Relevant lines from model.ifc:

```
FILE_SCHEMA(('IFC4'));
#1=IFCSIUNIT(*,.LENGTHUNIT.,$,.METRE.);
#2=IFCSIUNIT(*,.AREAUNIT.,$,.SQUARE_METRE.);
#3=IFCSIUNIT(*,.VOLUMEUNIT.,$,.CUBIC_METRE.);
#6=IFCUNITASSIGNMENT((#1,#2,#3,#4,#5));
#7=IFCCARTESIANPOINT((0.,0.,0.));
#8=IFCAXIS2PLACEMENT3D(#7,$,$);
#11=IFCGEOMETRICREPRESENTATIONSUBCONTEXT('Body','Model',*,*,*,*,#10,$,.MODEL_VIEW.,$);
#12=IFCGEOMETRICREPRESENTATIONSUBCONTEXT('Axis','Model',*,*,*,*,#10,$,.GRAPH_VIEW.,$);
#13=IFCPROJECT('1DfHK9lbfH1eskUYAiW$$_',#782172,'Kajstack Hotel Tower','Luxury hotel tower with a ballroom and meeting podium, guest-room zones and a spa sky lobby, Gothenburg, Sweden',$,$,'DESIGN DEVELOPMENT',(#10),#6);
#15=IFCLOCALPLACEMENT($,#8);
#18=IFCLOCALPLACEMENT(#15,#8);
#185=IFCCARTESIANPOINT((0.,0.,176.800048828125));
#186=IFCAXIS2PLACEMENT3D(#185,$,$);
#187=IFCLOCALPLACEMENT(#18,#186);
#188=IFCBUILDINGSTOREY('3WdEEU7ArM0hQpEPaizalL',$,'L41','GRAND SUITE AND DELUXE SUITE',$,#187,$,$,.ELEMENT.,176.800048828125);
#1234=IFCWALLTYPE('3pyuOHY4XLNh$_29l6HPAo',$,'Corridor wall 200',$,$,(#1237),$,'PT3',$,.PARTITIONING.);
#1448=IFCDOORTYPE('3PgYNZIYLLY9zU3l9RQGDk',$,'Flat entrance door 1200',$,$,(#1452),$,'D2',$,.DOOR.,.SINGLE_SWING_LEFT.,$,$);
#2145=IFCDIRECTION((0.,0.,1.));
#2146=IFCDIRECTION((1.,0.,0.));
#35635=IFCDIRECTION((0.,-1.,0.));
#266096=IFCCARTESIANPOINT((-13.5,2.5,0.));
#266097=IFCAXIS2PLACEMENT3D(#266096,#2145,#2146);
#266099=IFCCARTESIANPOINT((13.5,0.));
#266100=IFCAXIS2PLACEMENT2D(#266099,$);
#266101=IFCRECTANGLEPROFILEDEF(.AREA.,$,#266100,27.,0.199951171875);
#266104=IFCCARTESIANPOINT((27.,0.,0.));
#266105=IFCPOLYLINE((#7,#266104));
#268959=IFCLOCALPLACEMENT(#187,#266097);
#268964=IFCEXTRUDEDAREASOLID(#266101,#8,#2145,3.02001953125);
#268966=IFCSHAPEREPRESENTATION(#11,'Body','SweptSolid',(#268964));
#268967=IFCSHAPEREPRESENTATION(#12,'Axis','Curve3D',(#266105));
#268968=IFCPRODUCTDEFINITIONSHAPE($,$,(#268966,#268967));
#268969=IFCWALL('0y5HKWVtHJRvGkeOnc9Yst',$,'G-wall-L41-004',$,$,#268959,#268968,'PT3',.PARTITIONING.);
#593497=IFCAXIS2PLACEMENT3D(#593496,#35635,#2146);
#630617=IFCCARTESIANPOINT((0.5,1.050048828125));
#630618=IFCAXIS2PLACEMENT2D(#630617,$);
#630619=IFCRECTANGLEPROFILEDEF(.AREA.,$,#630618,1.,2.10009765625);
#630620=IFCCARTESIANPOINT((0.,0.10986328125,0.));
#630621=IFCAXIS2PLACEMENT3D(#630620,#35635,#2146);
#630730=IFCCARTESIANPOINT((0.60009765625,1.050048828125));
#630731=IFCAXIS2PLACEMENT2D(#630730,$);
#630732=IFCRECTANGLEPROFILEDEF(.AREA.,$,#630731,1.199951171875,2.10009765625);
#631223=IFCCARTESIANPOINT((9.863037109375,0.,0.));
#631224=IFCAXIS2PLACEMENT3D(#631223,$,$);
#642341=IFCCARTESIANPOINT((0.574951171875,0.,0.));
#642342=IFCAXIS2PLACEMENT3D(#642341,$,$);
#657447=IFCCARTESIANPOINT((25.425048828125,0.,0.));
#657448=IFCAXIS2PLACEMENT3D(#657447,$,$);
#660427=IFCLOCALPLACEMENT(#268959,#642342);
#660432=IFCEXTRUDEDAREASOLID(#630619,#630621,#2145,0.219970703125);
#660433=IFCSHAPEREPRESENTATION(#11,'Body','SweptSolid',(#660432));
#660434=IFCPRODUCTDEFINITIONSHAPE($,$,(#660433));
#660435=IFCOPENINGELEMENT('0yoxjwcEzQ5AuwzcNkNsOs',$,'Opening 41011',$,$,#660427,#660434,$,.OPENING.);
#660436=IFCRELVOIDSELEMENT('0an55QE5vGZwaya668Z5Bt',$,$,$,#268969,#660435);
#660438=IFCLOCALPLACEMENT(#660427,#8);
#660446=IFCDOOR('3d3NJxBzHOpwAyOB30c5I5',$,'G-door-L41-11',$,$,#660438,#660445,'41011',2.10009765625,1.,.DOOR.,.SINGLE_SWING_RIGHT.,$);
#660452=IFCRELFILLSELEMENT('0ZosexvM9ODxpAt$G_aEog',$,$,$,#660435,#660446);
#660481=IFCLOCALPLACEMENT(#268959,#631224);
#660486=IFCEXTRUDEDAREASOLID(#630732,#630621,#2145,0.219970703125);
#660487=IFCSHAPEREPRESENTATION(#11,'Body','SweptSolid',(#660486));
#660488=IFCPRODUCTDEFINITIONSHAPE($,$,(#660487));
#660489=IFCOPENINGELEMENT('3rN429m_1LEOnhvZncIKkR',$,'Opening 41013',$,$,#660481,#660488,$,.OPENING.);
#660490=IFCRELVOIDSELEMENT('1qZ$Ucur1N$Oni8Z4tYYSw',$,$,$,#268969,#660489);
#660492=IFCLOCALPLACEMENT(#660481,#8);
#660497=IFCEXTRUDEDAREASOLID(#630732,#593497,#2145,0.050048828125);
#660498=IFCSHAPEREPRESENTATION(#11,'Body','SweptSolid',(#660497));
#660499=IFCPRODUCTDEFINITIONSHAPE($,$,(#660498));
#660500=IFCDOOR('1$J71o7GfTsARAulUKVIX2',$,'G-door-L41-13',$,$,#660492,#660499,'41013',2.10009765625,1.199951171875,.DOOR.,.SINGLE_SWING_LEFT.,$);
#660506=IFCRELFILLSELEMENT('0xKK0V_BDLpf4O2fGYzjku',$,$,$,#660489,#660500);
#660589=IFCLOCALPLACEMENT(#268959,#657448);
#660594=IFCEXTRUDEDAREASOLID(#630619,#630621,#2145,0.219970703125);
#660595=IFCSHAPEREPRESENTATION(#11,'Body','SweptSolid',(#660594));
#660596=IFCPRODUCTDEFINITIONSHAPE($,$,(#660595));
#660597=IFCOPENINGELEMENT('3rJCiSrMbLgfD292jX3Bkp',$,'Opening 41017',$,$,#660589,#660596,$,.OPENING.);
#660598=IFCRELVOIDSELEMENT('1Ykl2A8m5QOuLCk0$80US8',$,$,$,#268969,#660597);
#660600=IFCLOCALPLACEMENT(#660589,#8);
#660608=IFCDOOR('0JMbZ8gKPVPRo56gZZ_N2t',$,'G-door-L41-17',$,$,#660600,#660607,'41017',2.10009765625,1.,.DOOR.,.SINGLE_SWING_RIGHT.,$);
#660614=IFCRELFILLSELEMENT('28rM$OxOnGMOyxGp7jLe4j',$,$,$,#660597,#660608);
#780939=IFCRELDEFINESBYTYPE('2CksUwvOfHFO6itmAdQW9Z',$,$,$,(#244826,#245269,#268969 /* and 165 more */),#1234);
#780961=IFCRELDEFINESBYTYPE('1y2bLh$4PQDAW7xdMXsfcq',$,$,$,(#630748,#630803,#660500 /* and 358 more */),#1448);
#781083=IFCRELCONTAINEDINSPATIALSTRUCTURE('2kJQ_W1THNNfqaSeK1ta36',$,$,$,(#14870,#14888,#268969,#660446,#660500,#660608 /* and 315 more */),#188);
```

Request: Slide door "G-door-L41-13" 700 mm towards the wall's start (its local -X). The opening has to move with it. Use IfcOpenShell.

```python
import ifcopenshell
import ifcopenshell.api.geometry
import ifcopenshell.util.placement
import ifcopenshell.util.unit

model = ifcopenshell.open("model.ifc")
unit_scale = ifcopenshell.util.unit.calculate_unit_scale(model)

door = model.by_id(660500)
opening = door.FillsVoids[0].RelatingOpeningElement
wall = opening.VoidsElements[0].RelatingBuildingElement

wall_matrix = ifcopenshell.util.placement.get_local_placement(wall.ObjectPlacement)
shift = wall_matrix[:3, 0] * -0.7 / unit_scale
before = ifcopenshell.util.placement.get_local_placement(door.ObjectPlacement)[:3, 3].copy()

# The door is placed relative to its opening, so it follows when the opening moves.
matrix = ifcopenshell.util.placement.get_local_placement(opening.ObjectPlacement)
matrix[:3, 3] += shift
ifcopenshell.api.geometry.edit_object_placement(
    model, product=opening, matrix=matrix, is_si=False, should_transform_children=True
)

after = ifcopenshell.util.placement.get_local_placement(door.ObjectPlacement)[:3, 3]
print("door moved by", (after - before).round(3) + 0.0)

model.write("model-out.ifc")
```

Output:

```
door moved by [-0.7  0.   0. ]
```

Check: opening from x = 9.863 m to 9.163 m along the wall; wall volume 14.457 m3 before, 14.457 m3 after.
